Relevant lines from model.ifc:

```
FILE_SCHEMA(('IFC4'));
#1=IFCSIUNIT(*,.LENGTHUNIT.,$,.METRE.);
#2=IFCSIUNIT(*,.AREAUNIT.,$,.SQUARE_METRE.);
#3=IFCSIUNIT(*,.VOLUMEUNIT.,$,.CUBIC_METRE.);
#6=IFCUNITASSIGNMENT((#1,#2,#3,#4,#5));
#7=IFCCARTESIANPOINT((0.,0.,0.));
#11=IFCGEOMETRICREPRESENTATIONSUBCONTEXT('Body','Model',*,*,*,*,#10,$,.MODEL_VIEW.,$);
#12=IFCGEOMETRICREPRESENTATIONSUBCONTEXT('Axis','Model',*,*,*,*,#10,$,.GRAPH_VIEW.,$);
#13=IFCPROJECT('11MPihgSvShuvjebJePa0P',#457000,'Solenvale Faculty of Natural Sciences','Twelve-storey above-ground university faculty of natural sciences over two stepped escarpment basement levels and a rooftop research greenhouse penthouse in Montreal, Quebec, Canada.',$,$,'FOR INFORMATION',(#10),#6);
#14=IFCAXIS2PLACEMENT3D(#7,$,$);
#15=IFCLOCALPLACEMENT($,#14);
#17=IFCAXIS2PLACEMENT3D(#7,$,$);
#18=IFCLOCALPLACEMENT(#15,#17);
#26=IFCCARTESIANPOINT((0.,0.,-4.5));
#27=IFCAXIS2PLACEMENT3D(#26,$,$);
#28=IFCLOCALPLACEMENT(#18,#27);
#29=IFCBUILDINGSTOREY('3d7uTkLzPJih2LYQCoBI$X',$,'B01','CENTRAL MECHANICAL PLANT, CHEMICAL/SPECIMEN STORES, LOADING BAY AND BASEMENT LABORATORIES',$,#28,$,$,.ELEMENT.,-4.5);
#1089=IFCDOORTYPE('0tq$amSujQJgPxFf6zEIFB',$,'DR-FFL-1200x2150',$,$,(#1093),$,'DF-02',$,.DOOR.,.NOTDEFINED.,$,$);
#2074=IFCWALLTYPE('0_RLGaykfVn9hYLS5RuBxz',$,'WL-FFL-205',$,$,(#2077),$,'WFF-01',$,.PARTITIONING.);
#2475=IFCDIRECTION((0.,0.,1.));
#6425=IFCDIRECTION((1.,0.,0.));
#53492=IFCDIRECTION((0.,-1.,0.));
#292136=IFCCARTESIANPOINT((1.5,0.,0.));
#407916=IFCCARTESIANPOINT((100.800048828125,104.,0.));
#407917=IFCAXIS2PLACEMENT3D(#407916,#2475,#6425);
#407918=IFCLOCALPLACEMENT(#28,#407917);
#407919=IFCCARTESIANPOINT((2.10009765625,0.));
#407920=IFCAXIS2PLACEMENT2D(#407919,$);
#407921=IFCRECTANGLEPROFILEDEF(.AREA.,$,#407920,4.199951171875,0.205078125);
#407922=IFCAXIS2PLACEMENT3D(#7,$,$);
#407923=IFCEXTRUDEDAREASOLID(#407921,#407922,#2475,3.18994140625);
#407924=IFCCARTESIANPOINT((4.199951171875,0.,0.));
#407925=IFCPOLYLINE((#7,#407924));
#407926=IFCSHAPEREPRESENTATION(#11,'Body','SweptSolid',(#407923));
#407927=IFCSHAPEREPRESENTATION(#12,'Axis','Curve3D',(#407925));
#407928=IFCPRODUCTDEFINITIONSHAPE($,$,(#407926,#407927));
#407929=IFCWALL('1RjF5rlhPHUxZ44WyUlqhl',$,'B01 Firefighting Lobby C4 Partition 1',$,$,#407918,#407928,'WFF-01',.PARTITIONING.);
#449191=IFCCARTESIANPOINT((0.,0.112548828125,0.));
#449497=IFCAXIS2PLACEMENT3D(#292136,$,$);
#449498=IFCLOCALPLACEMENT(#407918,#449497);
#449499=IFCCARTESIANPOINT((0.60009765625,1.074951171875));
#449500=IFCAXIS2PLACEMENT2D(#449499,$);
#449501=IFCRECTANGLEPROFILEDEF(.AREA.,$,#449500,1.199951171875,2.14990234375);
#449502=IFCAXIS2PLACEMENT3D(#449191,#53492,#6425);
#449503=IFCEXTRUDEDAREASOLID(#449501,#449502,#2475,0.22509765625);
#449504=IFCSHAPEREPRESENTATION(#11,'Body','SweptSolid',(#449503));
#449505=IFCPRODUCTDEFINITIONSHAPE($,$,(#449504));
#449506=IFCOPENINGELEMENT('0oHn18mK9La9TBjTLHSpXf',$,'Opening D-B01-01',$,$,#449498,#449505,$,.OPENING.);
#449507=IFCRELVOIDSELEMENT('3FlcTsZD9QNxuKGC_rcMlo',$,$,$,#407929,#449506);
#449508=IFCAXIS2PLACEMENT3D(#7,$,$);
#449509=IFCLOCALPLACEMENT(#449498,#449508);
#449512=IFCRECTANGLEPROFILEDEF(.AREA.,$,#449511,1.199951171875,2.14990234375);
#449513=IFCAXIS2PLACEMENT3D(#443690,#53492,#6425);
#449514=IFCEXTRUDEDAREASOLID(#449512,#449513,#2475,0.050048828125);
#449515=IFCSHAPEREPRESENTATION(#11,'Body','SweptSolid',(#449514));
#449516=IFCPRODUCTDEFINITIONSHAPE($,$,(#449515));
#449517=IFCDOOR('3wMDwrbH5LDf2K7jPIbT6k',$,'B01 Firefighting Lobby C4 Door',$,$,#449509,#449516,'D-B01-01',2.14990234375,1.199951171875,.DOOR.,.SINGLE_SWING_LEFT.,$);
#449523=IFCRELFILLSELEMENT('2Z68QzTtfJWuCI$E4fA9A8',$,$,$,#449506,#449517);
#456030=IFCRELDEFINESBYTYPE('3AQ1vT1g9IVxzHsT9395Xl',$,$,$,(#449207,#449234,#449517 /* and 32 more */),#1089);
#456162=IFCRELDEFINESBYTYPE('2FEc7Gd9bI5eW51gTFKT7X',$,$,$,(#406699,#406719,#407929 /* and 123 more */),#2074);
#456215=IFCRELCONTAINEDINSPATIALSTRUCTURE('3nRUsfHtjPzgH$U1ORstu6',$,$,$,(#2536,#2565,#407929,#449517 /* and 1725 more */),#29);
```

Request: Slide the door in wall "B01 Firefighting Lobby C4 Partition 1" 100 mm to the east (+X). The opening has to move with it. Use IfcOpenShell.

```python
import ifcopenshell
import ifcopenshell.api.geometry
import ifcopenshell.util.placement

model = ifcopenshell.open("model.ifc")

door = model.by_guid("3wMDwrbH5LDf2K7jPIbT6k")
opening = door.FillsVoids[0].RelatingOpeningElement
wall = opening.VoidsElements[0].RelatingBuildingElement

wall_matrix = ifcopenshell.util.placement.get_local_placement(wall.ObjectPlacement)
shift = wall_matrix[:3, 0] * 0.1
before = ifcopenshell.util.placement.get_local_placement(door.ObjectPlacement)[:3, 3].copy()

# The door is placed relative to its opening, so it follows when the opening moves.
matrix = ifcopenshell.util.placement.get_local_placement(opening.ObjectPlacement)
matrix[:3, 3] += shift
ifcopenshell.api.geometry.edit_object_placement(
    model, product=opening, matrix=matrix, is_si=False, should_transform_children=True
)

after = ifcopenshell.util.placement.get_local_placement(door.ObjectPlacement)[:3, 3]
print("door moved by", (after - before).round(3) + 0.0)

model.write("model_v2.ifc")
```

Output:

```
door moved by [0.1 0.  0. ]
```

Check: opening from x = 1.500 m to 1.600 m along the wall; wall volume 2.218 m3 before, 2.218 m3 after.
